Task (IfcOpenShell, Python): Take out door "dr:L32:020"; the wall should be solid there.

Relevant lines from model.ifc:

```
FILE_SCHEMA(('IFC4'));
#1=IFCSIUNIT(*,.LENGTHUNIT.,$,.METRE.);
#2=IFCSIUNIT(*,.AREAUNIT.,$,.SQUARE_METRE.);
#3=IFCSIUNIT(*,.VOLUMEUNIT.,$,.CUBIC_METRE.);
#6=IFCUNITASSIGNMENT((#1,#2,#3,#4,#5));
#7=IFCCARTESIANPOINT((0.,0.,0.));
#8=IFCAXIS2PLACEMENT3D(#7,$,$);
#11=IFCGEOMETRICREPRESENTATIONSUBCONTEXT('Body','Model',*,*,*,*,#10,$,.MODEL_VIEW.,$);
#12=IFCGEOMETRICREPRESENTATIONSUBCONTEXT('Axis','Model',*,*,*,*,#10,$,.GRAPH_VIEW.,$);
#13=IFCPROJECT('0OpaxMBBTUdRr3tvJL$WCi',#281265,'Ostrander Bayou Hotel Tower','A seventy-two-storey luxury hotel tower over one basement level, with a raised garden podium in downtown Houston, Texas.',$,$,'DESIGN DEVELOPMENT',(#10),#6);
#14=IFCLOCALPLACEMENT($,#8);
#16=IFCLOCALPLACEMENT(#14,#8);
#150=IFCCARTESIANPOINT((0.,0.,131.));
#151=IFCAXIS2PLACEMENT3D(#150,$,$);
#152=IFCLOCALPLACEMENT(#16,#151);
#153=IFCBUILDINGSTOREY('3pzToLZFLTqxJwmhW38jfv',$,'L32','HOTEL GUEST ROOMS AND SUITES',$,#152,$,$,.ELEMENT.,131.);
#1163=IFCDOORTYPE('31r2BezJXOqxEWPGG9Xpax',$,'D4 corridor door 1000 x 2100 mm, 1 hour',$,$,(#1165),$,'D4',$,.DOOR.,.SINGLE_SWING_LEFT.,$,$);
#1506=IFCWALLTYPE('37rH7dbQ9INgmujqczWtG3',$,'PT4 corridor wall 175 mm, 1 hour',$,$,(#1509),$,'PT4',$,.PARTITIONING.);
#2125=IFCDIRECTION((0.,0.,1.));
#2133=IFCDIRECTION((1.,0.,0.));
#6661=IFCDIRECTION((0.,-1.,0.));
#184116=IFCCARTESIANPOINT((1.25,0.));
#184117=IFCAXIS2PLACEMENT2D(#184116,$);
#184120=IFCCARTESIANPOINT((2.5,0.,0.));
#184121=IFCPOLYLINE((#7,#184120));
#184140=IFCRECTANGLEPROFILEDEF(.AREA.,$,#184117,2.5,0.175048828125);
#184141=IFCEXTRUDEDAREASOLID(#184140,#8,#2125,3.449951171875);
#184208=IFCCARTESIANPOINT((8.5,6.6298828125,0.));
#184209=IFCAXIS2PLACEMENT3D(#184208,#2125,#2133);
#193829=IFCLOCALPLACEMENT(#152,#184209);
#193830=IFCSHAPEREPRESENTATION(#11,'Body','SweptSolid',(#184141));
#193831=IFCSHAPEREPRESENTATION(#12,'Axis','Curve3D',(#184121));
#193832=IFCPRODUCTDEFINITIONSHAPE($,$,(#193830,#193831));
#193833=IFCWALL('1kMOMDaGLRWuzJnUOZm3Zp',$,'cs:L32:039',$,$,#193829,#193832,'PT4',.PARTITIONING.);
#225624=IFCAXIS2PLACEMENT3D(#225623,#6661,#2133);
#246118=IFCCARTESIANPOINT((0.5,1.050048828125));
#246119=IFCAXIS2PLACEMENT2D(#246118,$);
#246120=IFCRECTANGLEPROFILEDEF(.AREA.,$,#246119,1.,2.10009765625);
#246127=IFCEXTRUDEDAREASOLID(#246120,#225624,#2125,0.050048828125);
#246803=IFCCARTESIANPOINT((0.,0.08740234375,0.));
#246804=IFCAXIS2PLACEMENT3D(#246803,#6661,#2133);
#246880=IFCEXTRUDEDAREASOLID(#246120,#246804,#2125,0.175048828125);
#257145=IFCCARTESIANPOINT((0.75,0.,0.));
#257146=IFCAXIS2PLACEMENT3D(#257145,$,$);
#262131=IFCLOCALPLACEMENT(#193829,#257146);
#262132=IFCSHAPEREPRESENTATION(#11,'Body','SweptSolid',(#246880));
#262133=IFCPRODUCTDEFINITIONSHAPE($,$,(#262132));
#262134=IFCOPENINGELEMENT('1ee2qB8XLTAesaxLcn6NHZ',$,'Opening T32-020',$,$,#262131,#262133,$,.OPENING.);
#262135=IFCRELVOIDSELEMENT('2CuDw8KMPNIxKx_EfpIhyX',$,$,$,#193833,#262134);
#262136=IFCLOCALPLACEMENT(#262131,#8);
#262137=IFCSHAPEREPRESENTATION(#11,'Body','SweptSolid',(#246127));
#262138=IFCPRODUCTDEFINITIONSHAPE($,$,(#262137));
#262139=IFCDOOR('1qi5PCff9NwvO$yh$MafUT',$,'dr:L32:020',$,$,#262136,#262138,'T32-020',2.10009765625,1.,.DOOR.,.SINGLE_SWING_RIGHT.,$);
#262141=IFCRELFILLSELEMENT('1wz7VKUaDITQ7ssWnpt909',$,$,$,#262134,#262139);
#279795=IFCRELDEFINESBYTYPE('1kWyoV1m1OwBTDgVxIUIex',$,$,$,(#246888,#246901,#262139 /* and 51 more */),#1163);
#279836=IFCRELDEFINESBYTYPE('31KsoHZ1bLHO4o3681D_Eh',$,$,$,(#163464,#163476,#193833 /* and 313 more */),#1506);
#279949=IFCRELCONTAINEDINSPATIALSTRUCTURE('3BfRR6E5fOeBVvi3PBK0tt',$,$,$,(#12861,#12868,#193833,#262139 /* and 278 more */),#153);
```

```python
import ifcopenshell
import ifcopenshell.api.feature
import ifcopenshell.api.root
import ifcopenshell.geom
import ifcopenshell.util.shape

model = ifcopenshell.open("model.ifc")
settings = ifcopenshell.geom.settings()


def volume(element):
    """Net volume in cubic metres, openings subtracted."""
    shape = ifcopenshell.geom.create_shape(settings, element)
    return ifcopenshell.util.shape.get_volume(shape.geometry)


door = model.by_guid("1qi5PCff9NwvO$yh$MafUT")
opening = door.FillsVoids[0].RelatingOpeningElement
wall = opening.VoidsElements[0].RelatingBuildingElement
before = volume(wall)

ifcopenshell.api.root.remove_product(model, product=door)
ifcopenshell.api.feature.remove_feature(model, feature=opening)

after = volume(wall)

print(f"wall volume {before:.3f} -> {after:.3f} m3")

model.write("model-out.ifc")
```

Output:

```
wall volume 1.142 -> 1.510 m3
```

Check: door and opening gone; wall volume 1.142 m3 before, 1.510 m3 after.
